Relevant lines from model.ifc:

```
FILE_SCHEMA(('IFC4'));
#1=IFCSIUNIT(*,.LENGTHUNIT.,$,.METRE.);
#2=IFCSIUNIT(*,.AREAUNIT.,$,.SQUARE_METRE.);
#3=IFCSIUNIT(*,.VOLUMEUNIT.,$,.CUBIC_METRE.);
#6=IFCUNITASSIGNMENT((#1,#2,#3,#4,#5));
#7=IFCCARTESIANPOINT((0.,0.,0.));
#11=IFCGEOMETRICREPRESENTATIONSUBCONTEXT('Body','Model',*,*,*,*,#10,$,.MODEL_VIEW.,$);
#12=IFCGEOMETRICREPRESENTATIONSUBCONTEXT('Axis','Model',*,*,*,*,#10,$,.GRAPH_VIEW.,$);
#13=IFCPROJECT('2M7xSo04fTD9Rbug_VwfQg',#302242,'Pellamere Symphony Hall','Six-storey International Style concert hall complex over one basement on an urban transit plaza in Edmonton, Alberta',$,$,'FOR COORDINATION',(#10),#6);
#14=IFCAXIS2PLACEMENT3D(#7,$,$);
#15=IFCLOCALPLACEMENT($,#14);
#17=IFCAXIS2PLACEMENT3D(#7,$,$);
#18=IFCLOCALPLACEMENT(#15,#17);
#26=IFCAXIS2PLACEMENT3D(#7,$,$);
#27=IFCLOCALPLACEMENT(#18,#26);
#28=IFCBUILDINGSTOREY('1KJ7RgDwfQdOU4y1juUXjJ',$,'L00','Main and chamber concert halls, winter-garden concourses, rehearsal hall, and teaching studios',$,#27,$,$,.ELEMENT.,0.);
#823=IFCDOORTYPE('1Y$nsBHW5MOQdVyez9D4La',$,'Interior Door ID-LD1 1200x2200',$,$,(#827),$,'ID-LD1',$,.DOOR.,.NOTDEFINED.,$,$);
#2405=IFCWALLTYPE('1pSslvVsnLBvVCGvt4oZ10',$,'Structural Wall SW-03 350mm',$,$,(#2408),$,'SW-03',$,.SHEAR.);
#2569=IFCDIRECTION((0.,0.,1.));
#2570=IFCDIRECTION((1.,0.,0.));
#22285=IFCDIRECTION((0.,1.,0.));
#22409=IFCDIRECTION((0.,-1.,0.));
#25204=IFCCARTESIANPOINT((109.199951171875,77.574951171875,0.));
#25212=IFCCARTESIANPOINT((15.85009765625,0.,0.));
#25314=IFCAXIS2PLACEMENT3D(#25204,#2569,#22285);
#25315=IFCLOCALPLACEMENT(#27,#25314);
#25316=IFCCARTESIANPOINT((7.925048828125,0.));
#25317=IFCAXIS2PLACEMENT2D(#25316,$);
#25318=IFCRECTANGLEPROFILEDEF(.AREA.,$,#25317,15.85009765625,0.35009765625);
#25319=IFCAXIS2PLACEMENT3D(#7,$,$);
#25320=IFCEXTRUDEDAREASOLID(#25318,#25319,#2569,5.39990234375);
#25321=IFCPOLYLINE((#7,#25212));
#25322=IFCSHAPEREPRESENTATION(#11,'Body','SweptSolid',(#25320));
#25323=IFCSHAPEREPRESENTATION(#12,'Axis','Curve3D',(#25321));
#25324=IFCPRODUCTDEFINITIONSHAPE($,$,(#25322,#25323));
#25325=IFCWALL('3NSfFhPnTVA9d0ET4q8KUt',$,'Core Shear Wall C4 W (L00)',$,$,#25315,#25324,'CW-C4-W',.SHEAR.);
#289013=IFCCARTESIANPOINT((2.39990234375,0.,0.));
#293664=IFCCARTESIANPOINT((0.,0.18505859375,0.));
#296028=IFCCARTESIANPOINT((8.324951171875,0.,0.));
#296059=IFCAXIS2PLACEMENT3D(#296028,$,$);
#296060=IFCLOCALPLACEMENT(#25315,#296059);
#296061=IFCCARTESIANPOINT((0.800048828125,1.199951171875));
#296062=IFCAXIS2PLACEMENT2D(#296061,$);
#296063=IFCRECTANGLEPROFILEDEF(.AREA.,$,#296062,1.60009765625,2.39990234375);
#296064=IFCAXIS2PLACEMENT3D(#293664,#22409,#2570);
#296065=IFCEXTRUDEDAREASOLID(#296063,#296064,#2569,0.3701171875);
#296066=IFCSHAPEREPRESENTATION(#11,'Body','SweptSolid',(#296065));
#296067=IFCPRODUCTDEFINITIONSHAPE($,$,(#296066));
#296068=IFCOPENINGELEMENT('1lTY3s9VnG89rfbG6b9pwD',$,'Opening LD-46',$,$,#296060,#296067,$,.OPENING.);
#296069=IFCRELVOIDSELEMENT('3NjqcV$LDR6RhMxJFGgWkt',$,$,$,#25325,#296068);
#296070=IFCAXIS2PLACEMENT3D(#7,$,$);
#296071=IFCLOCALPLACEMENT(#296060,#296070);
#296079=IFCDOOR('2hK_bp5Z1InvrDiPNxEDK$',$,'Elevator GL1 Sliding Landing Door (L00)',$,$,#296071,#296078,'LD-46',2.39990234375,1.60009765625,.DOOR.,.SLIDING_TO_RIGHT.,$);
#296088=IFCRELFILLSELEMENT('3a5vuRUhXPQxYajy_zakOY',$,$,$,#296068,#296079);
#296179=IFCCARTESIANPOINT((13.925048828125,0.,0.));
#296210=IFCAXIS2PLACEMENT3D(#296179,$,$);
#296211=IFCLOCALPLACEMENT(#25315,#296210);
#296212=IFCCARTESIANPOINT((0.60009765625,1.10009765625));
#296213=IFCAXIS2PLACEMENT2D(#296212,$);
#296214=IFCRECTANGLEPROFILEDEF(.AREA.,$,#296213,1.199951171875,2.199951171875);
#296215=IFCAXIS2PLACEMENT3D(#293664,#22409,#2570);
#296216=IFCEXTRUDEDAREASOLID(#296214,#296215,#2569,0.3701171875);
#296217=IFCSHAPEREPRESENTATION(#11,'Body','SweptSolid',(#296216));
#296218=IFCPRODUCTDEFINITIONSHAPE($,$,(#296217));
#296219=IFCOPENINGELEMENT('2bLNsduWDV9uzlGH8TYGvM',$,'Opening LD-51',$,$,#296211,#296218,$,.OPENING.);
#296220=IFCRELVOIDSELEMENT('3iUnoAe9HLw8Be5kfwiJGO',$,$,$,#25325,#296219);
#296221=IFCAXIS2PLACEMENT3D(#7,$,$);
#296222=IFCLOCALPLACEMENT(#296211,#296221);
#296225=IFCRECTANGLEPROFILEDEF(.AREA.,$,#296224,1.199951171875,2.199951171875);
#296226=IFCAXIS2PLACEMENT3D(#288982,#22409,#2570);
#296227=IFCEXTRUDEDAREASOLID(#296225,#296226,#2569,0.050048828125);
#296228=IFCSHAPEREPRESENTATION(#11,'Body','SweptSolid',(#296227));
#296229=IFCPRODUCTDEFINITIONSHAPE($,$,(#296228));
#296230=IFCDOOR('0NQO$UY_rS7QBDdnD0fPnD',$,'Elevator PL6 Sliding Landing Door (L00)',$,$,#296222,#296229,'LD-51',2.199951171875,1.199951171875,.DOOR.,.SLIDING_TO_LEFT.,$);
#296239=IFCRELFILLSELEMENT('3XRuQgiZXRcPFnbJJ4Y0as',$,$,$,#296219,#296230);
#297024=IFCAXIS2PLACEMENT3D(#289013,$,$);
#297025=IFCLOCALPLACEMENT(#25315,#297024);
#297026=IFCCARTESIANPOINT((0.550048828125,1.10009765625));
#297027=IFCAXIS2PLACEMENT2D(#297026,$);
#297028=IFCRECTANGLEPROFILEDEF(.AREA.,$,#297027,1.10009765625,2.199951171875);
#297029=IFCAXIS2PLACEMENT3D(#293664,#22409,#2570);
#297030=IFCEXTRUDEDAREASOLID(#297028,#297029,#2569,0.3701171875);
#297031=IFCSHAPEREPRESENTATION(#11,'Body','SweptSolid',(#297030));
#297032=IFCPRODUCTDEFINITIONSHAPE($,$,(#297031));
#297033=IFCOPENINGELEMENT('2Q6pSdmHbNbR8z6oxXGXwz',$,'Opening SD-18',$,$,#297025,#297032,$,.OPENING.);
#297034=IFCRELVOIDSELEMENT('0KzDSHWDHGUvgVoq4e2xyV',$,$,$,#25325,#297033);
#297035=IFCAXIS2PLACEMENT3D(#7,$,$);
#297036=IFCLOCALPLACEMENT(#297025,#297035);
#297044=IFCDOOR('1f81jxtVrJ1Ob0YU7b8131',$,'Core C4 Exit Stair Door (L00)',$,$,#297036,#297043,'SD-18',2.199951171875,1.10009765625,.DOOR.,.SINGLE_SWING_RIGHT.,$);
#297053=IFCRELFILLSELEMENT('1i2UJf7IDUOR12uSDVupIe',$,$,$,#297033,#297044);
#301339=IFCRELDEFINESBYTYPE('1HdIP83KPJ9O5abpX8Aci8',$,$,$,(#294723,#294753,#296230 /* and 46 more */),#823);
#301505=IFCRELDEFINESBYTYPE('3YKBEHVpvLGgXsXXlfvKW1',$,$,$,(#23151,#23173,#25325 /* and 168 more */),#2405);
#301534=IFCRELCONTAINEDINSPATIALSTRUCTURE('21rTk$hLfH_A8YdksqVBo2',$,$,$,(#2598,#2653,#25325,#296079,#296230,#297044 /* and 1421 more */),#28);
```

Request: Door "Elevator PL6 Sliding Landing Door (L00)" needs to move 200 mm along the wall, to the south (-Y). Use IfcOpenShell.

```python
import ifcopenshell
import ifcopenshell.api.geometry
import ifcopenshell.util.placement
import ifcopenshell.util.unit

model = ifcopenshell.open("model.ifc")
unit_scale = ifcopenshell.util.unit.calculate_unit_scale(model)

door = model.by_id(296230)
opening = door.FillsVoids[0].RelatingOpeningElement
wall = opening.VoidsElements[0].RelatingBuildingElement

wall_matrix = ifcopenshell.util.placement.get_local_placement(wall.ObjectPlacement)
shift = wall_matrix[:3, 0] * -0.2 / unit_scale
before = ifcopenshell.util.placement.get_local_placement(door.ObjectPlacement)[:3, 3].copy()

# The door is placed relative to its opening, so it follows when the opening moves.
matrix = ifcopenshell.util.placement.get_local_placement(opening.ObjectPlacement)
matrix[:3, 3] += shift
ifcopenshell.api.geometry.edit_object_placement(
    model, product=opening, matrix=matrix, is_si=False, should_transform_children=True
)

after = ifcopenshell.util.placement.get_local_placement(door.ObjectPlacement)[:3, 3]
print("door moved by", (after - before).round(3) + 0.0)

model.write("model_edited.ifc")
```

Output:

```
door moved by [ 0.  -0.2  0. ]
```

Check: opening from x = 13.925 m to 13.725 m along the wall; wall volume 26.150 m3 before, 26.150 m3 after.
